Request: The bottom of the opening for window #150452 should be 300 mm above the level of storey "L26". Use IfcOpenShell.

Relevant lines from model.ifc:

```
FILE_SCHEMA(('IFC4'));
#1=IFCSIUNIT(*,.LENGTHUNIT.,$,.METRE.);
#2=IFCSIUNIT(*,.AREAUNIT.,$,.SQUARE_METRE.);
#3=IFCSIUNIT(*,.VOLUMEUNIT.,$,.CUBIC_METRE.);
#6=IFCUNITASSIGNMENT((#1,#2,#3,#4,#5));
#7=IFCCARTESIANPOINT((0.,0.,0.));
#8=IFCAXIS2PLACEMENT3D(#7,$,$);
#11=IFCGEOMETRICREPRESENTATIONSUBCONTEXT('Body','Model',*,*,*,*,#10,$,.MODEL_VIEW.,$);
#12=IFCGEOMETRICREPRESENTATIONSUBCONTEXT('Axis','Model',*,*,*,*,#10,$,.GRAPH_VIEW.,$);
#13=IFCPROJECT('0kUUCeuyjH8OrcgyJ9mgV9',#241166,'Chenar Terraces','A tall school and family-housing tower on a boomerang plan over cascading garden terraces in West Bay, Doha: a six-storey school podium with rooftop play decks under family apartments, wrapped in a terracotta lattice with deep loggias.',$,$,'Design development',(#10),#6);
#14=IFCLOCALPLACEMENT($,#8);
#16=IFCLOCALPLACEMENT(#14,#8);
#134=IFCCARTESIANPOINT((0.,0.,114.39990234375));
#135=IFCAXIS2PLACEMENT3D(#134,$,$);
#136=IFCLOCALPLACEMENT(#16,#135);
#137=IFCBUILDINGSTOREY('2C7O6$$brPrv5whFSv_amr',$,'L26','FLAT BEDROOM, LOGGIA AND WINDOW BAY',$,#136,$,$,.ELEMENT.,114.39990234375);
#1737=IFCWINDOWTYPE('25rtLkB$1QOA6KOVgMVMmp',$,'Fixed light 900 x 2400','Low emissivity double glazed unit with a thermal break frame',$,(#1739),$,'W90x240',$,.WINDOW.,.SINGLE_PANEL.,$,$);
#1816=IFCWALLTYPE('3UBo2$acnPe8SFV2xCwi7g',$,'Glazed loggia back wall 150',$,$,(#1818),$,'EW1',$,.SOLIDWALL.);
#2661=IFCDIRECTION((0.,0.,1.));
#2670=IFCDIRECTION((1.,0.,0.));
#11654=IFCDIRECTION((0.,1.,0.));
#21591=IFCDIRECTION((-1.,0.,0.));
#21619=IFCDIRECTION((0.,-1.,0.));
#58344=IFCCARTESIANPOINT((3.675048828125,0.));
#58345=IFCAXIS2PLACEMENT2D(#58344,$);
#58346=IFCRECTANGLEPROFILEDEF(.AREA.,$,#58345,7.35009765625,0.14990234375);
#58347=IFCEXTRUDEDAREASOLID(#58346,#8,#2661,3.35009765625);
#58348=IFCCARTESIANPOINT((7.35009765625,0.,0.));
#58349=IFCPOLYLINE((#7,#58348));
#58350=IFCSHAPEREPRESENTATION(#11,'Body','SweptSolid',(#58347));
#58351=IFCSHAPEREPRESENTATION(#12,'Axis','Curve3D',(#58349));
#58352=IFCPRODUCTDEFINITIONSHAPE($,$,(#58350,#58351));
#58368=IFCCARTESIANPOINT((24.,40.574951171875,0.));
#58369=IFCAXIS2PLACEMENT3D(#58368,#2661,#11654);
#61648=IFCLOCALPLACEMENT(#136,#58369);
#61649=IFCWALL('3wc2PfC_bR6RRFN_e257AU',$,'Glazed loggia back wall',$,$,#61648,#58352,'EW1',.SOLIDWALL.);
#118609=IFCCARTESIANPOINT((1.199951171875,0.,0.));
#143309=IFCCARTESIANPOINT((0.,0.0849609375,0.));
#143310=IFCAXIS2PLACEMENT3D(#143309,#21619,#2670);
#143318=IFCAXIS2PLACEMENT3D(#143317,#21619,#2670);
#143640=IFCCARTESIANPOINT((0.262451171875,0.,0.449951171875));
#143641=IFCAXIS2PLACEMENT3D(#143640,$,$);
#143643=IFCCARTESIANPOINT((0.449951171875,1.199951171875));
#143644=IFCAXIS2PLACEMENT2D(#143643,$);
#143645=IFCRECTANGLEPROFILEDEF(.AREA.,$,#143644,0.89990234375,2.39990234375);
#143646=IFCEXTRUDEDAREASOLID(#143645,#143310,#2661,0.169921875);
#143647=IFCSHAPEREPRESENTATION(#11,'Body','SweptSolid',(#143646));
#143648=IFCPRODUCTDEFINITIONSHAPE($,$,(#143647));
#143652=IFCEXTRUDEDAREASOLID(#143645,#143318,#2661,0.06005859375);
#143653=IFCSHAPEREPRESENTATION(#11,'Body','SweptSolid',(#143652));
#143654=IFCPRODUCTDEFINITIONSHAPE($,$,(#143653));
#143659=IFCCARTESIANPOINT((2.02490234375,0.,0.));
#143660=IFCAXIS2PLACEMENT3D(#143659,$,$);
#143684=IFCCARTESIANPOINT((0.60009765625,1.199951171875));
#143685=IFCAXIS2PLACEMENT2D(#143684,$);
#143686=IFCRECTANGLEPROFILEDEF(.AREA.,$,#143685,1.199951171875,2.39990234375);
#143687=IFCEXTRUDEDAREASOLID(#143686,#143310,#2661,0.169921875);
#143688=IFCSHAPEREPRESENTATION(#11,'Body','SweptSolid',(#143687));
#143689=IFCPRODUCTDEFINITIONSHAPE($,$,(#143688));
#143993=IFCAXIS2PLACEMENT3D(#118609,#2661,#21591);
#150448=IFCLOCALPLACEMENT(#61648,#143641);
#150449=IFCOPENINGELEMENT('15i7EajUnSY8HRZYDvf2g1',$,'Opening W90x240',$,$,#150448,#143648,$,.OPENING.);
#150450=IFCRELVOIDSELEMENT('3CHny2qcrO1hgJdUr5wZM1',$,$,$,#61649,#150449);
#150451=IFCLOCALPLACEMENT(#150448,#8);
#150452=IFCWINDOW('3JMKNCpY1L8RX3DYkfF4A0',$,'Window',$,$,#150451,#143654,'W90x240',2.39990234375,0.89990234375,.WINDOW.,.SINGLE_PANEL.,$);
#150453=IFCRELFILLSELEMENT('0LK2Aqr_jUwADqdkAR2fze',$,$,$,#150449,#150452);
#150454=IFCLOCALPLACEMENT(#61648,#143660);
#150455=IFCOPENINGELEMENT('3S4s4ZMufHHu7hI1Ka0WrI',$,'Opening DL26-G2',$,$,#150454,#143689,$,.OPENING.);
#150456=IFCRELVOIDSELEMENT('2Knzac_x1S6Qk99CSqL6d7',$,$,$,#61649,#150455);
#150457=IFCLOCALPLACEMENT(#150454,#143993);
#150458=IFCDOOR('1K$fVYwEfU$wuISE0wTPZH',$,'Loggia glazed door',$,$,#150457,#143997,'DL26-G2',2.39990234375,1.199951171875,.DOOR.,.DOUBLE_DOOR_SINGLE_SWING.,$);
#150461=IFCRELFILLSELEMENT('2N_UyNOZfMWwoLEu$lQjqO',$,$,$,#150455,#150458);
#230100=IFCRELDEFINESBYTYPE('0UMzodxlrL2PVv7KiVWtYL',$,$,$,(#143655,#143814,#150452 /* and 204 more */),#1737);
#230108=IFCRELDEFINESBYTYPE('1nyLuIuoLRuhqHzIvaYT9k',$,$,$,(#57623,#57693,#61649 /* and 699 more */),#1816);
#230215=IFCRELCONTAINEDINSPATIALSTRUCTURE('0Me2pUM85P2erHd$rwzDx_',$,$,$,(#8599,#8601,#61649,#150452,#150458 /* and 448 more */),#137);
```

```python
import numpy as np
import ifcopenshell
import ifcopenshell.api.geometry
import ifcopenshell.geom
import ifcopenshell.util.element
import ifcopenshell.util.placement
import ifcopenshell.util.shape
import ifcopenshell.util.unit

model = ifcopenshell.open("model.ifc")
unit_scale = ifcopenshell.util.unit.calculate_unit_scale(model)

window = model.by_guid("3JMKNCpY1L8RX3DYkfF4A0")
opening = window.FillsVoids[0].RelatingOpeningElement
storey = ifcopenshell.util.element.get_container(window, ifc_class="IfcBuildingStorey")
level = ifcopenshell.util.placement.get_local_placement(storey.ObjectPlacement)[2, 3]

# The opening's origin need not be at the sill, so measure its lowest point.
shape = ifcopenshell.geom.create_shape(ifcopenshell.geom.settings(), opening)
bottom = ifcopenshell.util.shape.get_shape_bottom_elevation(shape, shape.geometry) / unit_scale
dz = level + 0.3 - bottom

shift = np.array([0.0, 0.0, dz])
# The window is placed relative to its opening, so it follows when the opening moves.
matrix = ifcopenshell.util.placement.get_local_placement(opening.ObjectPlacement)
matrix[:3, 3] += shift
ifcopenshell.api.geometry.edit_object_placement(
    model, product=opening, matrix=matrix, is_si=False, should_transform_children=True
)

print(f"moved by {dz * unit_scale:+.3f} m")

model.write("model_v2.ifc")
```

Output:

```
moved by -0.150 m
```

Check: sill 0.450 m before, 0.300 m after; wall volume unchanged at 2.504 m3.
